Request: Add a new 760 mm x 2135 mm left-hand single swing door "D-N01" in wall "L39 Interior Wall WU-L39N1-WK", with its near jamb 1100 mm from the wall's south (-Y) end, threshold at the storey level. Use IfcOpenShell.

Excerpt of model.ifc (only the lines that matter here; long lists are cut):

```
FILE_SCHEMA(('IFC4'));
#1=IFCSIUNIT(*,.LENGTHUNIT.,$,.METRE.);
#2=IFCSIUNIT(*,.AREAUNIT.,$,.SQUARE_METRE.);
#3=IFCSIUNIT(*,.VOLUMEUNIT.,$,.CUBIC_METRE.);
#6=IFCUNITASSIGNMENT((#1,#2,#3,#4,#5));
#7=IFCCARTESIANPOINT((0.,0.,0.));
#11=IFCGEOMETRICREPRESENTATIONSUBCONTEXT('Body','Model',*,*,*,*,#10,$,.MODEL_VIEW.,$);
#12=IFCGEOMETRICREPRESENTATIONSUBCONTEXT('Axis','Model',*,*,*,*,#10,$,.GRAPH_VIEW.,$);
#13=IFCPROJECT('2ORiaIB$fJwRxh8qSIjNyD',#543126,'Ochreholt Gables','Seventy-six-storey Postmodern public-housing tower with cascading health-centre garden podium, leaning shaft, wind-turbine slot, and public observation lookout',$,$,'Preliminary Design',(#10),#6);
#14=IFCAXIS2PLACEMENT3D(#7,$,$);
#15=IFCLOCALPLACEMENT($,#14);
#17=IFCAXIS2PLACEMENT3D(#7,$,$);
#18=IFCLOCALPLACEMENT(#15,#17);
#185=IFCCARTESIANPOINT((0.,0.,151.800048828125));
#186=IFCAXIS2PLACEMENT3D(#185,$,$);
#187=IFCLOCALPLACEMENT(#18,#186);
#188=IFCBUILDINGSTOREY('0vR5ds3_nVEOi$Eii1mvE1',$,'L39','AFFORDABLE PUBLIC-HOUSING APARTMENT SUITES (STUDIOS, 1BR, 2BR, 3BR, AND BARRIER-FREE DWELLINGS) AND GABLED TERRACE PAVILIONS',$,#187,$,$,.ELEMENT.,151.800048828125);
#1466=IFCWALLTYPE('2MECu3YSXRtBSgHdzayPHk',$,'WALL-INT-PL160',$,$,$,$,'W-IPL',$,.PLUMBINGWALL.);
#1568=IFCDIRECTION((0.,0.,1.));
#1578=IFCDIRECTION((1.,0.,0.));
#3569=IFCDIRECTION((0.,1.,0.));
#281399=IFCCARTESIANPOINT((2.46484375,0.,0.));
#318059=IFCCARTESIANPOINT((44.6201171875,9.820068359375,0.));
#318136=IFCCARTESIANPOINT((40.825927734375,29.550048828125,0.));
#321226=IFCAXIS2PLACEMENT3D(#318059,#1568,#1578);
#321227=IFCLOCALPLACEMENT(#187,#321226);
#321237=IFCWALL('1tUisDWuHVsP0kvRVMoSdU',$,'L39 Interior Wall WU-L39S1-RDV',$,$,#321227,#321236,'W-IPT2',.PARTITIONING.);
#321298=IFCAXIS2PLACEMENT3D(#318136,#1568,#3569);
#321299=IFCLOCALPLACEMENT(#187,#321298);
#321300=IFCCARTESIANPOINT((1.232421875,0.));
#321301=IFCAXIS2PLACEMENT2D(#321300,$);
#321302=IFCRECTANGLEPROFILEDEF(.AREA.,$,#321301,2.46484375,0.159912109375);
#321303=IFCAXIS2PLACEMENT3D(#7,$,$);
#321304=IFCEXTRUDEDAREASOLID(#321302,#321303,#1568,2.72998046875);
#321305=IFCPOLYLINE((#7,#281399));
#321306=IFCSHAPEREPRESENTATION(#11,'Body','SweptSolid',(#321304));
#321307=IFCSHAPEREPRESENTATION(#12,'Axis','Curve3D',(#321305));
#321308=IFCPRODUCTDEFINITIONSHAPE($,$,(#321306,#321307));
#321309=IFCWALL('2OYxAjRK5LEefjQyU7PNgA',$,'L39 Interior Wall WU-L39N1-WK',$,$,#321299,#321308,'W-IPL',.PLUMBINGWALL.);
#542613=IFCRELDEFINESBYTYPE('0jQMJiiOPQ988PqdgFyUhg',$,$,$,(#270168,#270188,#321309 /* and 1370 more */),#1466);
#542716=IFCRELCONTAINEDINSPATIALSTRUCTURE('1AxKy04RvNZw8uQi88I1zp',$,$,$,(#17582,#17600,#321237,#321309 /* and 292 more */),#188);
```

```python
import numpy as np
import ifcopenshell
import ifcopenshell.api.feature
import ifcopenshell.api.geometry
import ifcopenshell.api.root
import ifcopenshell.api.spatial
import ifcopenshell.geom
import ifcopenshell.util.element
import ifcopenshell.util.placement
import ifcopenshell.util.representation
import ifcopenshell.util.shape
import ifcopenshell.util.unit

model = ifcopenshell.open("model.ifc")
unit_scale = ifcopenshell.util.unit.calculate_unit_scale(model)
settings = ifcopenshell.geom.settings()


def volume(element):
    """Net volume in cubic metres, openings subtracted."""
    shape = ifcopenshell.geom.create_shape(settings, element)
    return ifcopenshell.util.shape.get_volume(shape.geometry)


wall = model.by_guid("2OYxAjRK5LEefjQyU7PNgA")
storey = ifcopenshell.util.element.get_container(wall, ifc_class="IfcBuildingStorey")
context = ifcopenshell.util.representation.get_context(model, "Model", "Body", "MODEL_VIEW")
before = volume(wall)

width, height, from_end, sill = 0.76, 2.135, 1.1, 0.0  # metres

# The wall runs along its own X axis, and the end named is its -X end.
wall_shape = ifcopenshell.geom.create_shape(settings, wall)
x, y, z = ifcopenshell.util.shape.get_vertices(wall_shape.geometry).T
start = x.min() + from_end
face, thickness = float(y.min()), float(y.max() - y.min())
wall_matrix = ifcopenshell.util.placement.get_local_placement(wall.ObjectPlacement)
level = ifcopenshell.util.placement.get_local_placement(storey.ObjectPlacement)[2, 3]


def in_wall(x, y):
    """Placement at x, y metres in the wall's axes, at sill height."""
    matrix = wall_matrix.copy()
    matrix[:, 3] = wall_matrix @ np.array([x / unit_scale, y / unit_scale, 0.0, 1.0])
    matrix[2, 3] = level + sill / unit_scale
    return matrix


# Opening: a box that overshoots both wall faces by 50 mm.
opening = ifcopenshell.api.root.create_entity(model, ifc_class="IfcOpeningElement", predefined_type="OPENING")
box = ifcopenshell.api.geometry.add_wall_representation(
    model, context=context, length=width, height=height, thickness=thickness + 0.1
)
ifcopenshell.api.geometry.assign_representation(model, product=opening, representation=box)
ifcopenshell.api.geometry.edit_object_placement(model, product=opening, matrix=in_wall(start, face - 0.05), is_si=False)
ifcopenshell.api.feature.add_feature(model, feature=opening, element=wall)

door = ifcopenshell.api.root.create_entity(model, ifc_class="IfcDoor", name="D-N01", predefined_type="DOOR")
door.OverallWidth, door.OverallHeight = width / unit_scale, height / unit_scale
door.OperationType = "SINGLE_SWING_LEFT"
body = ifcopenshell.api.geometry.add_door_representation(
    model,
    context=context,
    overall_width=door.OverallWidth,
    overall_height=door.OverallHeight,
    operation_type="SINGLE_SWING_LEFT",
    lining_properties={"LiningDepth": thickness / unit_scale, "ThresholdDepth": thickness / unit_scale},
)
ifcopenshell.api.geometry.assign_representation(model, product=door, representation=body)
ifcopenshell.api.spatial.assign_container(model, products=[door], relating_structure=storey)
ifcopenshell.api.feature.add_filling(model, opening=opening, element=door)

# The lining spans the wall, so the door starts at the wall face.
ifcopenshell.api.geometry.edit_object_placement(model, product=door, matrix=in_wall(start, face), is_si=False)

after = volume(wall)

print(f"wall volume {before:.3f} -> {after:.3f} m3")

model.write("model_updated.ifc")
```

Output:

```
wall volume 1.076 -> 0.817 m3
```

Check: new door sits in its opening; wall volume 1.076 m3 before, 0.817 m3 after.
